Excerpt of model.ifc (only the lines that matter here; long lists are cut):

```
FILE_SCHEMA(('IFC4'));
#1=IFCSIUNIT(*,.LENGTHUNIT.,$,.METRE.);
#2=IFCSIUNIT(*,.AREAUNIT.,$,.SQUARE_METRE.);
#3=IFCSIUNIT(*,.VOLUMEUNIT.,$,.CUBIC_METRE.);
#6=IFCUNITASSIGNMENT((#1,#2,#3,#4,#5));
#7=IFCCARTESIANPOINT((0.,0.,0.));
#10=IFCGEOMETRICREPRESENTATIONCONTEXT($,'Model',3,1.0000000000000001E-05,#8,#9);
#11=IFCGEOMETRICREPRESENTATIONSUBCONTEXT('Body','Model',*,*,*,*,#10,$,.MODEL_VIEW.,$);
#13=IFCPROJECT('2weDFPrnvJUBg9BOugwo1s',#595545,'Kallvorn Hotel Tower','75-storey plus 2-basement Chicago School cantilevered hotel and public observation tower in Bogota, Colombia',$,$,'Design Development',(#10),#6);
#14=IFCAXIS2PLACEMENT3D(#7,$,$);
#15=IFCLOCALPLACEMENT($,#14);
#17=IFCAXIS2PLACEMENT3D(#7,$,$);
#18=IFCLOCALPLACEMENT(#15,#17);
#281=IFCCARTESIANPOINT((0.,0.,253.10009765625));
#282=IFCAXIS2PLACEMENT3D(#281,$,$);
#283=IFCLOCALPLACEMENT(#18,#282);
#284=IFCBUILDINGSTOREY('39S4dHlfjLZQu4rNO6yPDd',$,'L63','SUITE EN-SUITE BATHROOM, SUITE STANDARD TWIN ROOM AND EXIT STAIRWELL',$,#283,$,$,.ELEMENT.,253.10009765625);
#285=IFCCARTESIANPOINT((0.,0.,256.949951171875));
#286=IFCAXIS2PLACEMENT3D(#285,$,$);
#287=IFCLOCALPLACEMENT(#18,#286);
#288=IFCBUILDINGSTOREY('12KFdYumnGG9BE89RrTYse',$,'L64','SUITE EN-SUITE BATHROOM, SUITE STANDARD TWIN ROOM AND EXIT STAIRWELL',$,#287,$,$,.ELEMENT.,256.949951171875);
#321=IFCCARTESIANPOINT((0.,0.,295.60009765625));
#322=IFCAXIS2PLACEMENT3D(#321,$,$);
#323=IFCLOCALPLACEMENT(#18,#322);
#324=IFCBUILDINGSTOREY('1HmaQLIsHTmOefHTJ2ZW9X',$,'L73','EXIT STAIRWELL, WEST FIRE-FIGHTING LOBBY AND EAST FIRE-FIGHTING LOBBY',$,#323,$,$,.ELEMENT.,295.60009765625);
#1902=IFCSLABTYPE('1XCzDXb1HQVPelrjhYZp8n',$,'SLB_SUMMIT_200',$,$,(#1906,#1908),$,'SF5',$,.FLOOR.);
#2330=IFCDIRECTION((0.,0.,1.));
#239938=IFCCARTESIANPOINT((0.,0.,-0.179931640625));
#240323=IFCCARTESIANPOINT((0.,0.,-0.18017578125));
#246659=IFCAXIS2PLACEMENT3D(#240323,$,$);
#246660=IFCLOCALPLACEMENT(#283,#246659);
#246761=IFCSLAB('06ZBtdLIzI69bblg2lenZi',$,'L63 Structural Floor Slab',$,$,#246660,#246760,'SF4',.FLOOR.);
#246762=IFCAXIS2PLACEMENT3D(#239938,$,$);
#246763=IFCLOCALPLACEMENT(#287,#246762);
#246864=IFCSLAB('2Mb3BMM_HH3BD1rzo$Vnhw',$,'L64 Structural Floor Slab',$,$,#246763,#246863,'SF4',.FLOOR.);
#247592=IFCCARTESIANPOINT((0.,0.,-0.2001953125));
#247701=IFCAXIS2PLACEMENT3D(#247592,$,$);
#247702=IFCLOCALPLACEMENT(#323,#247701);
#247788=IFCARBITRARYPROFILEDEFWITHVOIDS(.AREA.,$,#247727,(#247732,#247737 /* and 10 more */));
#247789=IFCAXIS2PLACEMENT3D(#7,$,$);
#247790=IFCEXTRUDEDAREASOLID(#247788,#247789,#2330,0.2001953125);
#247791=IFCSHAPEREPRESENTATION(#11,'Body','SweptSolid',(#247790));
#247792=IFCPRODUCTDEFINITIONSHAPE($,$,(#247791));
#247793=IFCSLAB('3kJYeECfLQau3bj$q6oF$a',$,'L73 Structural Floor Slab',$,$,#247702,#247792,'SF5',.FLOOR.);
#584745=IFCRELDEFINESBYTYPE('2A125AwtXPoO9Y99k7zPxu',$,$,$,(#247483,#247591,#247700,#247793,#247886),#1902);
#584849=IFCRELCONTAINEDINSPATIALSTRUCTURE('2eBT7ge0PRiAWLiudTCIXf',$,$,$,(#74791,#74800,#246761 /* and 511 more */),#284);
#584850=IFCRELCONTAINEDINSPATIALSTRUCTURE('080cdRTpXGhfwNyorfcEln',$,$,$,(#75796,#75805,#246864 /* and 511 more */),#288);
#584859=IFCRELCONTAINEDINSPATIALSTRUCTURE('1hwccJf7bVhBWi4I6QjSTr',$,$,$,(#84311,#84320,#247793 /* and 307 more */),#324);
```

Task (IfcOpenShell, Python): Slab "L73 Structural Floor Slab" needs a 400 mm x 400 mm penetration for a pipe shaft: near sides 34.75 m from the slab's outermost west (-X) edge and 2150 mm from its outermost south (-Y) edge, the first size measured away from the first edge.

```python
import numpy as np
import ifcopenshell
import ifcopenshell.api.feature
import ifcopenshell.api.geometry
import ifcopenshell.api.root
import ifcopenshell.geom
import ifcopenshell.util.placement
import ifcopenshell.util.representation
import ifcopenshell.util.shape
import ifcopenshell.util.unit

model = ifcopenshell.open("model.ifc")
unit_scale = ifcopenshell.util.unit.calculate_unit_scale(model)
settings = ifcopenshell.geom.settings()


def volume(element):
    """Net volume in cubic metres, openings subtracted."""
    shape = ifcopenshell.geom.create_shape(settings, element)
    return ifcopenshell.util.shape.get_volume(shape.geometry)


slab = model.by_id(247793)
before = volume(slab)

# Extent in the slab's own axes, in metres. The edges named are its -X and -Y sides.
slab_shape = ifcopenshell.geom.create_shape(settings, slab)
vertices = ifcopenshell.util.shape.get_vertices(slab_shape.geometry)
x_min, y_min, bottom = vertices.min(axis=0)
top = vertices[:, 2].max()

opening = ifcopenshell.api.root.create_entity(model, ifc_class="IfcOpeningElement", name="Pipe shaft opening", predefined_type="OPENING")
context = ifcopenshell.util.representation.get_context(model, "Model", "Body", "MODEL_VIEW")
width, depth = 0.4, 0.4
outline = [(0.0, 0.0), (width, 0.0), (width, depth), (0.0, depth), (0.0, 0.0)]
# Overshoot both faces by 50 mm so the cut is clean.
shape = ifcopenshell.api.geometry.add_slab_representation(
    model, context=context, depth=top - bottom + 0.1, polyline=outline
)
ifcopenshell.api.geometry.assign_representation(model, product=opening, representation=shape)

matrix = ifcopenshell.util.placement.get_local_placement(slab.ObjectPlacement)
matrix[:, 3] = matrix @ np.append(np.array([x_min + 34.75, y_min + 2.15, bottom - 0.05]) / unit_scale, 1.0)
ifcopenshell.api.geometry.edit_object_placement(model, product=opening, matrix=matrix, is_si=False)
ifcopenshell.api.feature.add_feature(model, feature=opening, element=slab)

after = volume(slab)

print(f"slab volume {before:.3f} -> {after:.3f} m3")

model.write("model_updated.ifc")
```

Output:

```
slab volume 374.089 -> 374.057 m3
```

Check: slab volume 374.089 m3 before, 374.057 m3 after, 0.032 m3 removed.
